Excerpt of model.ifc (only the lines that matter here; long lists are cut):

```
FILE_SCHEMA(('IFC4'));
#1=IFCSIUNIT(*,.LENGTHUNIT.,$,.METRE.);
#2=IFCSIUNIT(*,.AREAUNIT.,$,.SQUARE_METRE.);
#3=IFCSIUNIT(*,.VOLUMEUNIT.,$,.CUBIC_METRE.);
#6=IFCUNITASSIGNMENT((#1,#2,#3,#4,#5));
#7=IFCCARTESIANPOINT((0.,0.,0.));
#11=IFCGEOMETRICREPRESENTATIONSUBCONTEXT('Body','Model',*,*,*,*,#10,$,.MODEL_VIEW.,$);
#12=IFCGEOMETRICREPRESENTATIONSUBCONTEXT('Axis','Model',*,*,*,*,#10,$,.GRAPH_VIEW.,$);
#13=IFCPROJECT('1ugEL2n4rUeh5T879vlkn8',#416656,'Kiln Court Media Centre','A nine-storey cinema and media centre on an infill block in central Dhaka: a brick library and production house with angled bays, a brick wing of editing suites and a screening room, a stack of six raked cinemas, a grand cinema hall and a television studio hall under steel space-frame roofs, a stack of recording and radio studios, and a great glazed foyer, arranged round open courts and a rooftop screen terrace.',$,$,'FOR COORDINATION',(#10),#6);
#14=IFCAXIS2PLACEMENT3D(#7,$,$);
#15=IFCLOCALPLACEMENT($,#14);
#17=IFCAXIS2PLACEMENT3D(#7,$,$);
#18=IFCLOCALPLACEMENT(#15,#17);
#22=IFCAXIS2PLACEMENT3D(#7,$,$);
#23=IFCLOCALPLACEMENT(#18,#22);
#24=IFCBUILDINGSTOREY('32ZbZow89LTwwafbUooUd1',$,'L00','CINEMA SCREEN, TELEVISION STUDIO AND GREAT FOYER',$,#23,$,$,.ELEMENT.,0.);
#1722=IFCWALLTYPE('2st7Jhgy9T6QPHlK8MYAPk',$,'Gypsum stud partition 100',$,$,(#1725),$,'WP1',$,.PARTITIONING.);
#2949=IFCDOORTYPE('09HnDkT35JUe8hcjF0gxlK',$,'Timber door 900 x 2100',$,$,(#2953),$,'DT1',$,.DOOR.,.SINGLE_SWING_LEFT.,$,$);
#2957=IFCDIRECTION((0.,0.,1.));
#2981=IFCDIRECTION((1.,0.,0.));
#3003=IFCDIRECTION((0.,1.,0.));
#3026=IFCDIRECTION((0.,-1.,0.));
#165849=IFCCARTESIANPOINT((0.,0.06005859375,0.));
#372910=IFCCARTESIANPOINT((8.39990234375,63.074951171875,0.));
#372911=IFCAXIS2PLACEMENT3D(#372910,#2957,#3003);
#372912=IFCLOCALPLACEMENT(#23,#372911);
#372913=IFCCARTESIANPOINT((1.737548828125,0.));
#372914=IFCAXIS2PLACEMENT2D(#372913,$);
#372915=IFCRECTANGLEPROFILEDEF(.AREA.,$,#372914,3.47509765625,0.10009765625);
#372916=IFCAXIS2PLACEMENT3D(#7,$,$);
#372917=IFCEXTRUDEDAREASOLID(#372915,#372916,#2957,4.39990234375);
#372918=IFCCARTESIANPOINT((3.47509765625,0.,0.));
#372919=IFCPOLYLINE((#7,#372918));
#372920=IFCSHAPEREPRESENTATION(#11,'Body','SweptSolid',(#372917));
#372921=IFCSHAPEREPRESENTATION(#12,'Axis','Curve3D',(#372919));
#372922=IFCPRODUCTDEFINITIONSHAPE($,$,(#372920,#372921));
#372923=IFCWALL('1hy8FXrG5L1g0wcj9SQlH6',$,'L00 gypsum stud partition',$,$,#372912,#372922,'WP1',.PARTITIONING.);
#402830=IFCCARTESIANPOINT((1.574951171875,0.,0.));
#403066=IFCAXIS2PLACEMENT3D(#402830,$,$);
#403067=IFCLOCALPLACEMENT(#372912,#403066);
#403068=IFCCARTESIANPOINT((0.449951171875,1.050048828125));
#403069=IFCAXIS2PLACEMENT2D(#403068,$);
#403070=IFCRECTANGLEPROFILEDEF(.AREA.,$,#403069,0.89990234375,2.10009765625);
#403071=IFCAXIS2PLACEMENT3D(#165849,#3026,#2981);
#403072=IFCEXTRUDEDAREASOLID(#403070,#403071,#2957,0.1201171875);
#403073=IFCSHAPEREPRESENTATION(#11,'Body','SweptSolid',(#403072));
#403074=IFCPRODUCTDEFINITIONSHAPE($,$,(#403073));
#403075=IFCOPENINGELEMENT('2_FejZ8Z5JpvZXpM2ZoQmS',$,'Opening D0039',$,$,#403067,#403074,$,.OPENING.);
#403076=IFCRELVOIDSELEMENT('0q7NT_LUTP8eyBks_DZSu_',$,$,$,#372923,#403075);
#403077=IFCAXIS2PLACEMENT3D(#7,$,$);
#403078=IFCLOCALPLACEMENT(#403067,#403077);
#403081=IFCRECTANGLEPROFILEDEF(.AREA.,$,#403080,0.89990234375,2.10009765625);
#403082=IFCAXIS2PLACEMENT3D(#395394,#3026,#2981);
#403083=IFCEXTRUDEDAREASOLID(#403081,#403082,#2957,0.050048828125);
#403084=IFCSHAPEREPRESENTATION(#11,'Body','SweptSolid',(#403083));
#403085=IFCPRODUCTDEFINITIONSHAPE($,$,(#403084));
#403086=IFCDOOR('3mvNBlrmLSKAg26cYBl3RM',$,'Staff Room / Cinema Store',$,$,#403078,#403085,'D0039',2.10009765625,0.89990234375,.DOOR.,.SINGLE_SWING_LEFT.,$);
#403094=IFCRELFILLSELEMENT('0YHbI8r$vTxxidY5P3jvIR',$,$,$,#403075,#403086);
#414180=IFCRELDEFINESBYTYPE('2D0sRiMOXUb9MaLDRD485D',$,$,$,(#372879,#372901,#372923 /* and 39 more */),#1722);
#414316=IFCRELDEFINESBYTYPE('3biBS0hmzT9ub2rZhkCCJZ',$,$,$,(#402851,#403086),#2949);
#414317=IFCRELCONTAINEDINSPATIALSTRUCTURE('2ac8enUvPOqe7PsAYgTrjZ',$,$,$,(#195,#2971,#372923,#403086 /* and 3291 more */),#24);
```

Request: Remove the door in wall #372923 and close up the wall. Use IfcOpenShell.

```python
import ifcopenshell
import ifcopenshell.api.feature
import ifcopenshell.api.root
import ifcopenshell.geom
import ifcopenshell.util.shape

model = ifcopenshell.open("model.ifc")
settings = ifcopenshell.geom.settings()


def volume(element):
    """Net volume in cubic metres, openings subtracted."""
    shape = ifcopenshell.geom.create_shape(settings, element)
    return ifcopenshell.util.shape.get_volume(shape.geometry)


door = model.by_guid("3mvNBlrmLSKAg26cYBl3RM")
opening = door.FillsVoids[0].RelatingOpeningElement
wall = opening.VoidsElements[0].RelatingBuildingElement
before = volume(wall)

ifcopenshell.api.root.remove_product(model, product=door)
ifcopenshell.api.feature.remove_feature(model, feature=opening)

after = volume(wall)

print(f"wall volume {before:.3f} -> {after:.3f} m3")

model.write("model_v2.ifc")
```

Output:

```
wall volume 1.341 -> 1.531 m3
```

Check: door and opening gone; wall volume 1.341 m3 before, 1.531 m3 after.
